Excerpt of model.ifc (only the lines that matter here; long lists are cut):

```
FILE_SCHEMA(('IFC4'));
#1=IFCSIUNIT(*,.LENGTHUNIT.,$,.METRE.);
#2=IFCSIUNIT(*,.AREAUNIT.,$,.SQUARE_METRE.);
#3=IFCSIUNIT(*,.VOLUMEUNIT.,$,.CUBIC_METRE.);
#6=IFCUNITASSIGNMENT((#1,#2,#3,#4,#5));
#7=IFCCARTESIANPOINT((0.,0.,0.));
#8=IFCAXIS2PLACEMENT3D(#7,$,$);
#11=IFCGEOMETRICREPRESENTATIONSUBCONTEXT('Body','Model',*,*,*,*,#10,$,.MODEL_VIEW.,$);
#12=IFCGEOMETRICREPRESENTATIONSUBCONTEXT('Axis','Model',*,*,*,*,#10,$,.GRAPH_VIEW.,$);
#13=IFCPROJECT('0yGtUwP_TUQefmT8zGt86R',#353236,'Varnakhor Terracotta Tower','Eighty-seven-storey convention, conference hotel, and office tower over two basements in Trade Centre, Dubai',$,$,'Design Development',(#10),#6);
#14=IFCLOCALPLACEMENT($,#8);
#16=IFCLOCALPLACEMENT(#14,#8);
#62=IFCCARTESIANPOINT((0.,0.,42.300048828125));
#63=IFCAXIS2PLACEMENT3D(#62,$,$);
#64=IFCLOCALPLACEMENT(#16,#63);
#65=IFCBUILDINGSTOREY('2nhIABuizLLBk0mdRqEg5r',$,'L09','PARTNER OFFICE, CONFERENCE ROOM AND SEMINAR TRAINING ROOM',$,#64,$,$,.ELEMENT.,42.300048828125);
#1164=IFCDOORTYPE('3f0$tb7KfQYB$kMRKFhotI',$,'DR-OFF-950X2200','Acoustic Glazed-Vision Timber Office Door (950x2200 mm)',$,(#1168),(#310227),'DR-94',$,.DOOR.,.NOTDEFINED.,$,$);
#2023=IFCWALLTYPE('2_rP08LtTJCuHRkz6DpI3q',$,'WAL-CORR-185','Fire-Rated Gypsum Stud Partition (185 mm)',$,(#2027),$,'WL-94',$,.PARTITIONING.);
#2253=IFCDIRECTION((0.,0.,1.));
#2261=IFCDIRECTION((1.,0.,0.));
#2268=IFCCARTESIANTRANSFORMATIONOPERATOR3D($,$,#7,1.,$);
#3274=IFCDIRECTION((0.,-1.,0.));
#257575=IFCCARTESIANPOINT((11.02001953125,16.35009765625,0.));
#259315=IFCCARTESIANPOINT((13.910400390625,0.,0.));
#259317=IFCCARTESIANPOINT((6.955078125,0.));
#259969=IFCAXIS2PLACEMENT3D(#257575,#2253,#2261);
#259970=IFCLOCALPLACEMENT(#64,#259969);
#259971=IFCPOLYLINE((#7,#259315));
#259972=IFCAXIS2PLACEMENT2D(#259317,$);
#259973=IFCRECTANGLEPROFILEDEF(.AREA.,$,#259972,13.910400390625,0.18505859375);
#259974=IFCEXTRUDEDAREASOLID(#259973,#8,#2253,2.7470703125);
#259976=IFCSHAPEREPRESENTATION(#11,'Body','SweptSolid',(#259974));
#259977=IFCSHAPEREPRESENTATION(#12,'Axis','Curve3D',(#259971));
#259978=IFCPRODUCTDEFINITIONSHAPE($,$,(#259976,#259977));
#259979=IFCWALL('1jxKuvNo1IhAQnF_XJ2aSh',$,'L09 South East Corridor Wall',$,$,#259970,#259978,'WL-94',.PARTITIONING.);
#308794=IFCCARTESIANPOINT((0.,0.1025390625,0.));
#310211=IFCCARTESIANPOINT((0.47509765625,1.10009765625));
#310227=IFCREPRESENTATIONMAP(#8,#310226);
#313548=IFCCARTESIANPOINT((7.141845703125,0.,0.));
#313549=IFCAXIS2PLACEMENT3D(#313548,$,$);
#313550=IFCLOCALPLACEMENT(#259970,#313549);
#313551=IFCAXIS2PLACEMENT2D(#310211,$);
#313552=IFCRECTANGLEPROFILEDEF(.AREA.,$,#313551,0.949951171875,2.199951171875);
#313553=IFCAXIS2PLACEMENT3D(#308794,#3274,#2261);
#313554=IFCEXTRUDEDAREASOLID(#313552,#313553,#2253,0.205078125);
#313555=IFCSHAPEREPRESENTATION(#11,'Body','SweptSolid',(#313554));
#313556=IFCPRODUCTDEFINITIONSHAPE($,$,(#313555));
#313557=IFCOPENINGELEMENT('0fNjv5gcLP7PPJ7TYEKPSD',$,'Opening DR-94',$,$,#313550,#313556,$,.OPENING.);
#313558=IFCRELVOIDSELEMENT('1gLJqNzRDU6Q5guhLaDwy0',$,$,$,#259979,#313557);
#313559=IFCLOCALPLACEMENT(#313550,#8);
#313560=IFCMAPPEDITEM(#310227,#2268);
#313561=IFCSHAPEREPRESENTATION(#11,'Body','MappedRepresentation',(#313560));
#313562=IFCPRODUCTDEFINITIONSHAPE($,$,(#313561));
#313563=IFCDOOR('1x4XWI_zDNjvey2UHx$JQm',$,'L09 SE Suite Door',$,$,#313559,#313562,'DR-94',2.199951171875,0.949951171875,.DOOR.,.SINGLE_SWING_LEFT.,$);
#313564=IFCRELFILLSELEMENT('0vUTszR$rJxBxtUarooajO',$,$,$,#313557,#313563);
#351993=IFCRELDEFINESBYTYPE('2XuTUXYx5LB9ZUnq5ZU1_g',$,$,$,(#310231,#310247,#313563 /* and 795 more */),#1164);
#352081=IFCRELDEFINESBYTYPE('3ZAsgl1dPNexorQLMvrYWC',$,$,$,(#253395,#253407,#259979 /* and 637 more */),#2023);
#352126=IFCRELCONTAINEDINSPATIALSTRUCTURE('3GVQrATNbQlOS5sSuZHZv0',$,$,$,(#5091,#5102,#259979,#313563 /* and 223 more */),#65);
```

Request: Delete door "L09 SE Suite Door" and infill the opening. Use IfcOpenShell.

```python
import ifcopenshell
import ifcopenshell.api.feature
import ifcopenshell.api.root
import ifcopenshell.geom
import ifcopenshell.util.shape

model = ifcopenshell.open("model.ifc")
settings = ifcopenshell.geom.settings()


def volume(element):
    """Net volume in cubic metres, openings subtracted."""
    shape = ifcopenshell.geom.create_shape(settings, element)
    return ifcopenshell.util.shape.get_volume(shape.geometry)


door = model.by_guid("1x4XWI_zDNjvey2UHx$JQm")
opening = door.FillsVoids[0].RelatingOpeningElement
wall = opening.VoidsElements[0].RelatingBuildingElement
before = volume(wall)

ifcopenshell.api.root.remove_product(model, product=door)
ifcopenshell.api.feature.remove_feature(model, feature=opening)

after = volume(wall)

print(f"wall volume {before:.3f} -> {after:.3f} m3")

model.write("model_v2.ifc")
```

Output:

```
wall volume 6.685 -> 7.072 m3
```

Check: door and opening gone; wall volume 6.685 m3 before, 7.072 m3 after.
